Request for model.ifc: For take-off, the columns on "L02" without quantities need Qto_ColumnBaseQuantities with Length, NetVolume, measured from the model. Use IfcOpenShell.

First a look at what the model holds.

```python
import ifcopenshell
import ifcopenshell.util.element
import ifcopenshell.util.unit

model = ifcopenshell.open("model.ifc")
print(model.schema)
for unit_type in ("LENGTHUNIT", "AREAUNIT", "VOLUMEUNIT"):
    print(unit_type, ifcopenshell.util.unit.calculate_unit_scale(model, unit_type))
storey = next(s for s in model.by_type("IfcBuildingStorey") if s.Name == "L02")
columns = [e for e in ifcopenshell.util.element.get_decomposition(storey) if e.is_a("IfcColumn")]
for e in sorted(columns, key=lambda e: e.id()):
    print(e.id(), e.is_a(), e.Name, list(ifcopenshell.util.element.get_psets(e, qtos_only=True)), sep=" | ")
```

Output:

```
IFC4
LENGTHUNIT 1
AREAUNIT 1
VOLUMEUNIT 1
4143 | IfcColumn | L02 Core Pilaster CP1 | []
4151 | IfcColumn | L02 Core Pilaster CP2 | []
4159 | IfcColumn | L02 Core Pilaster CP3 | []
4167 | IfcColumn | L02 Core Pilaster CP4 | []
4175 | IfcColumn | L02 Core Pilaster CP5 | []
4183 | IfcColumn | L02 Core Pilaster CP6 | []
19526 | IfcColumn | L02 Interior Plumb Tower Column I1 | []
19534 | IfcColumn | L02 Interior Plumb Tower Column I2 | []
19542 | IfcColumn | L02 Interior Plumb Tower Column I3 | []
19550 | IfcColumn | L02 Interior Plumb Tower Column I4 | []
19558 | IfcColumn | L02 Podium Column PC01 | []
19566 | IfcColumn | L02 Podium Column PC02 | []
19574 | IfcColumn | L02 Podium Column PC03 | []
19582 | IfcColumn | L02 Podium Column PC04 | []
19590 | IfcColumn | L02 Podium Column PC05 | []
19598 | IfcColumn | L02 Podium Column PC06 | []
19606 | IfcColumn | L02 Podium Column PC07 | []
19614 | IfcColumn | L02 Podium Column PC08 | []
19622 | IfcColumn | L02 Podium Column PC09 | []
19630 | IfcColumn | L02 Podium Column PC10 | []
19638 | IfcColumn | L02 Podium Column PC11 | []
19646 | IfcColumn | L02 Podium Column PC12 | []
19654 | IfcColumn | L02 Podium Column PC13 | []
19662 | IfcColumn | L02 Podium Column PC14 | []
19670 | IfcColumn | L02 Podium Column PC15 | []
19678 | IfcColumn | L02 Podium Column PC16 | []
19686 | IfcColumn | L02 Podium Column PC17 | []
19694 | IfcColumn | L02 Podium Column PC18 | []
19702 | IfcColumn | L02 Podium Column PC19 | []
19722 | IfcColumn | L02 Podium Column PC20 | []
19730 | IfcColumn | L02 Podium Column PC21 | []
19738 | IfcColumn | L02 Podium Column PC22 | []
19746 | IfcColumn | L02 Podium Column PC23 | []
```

```python
import ifcopenshell
import ifcopenshell.api.pset
import ifcopenshell.geom
import ifcopenshell.util.element
import ifcopenshell.util.shape
import ifcopenshell.util.unit

model = ifcopenshell.open("model.ifc")
unit_scale = ifcopenshell.util.unit.calculate_unit_scale(model)
volume_scale = ifcopenshell.util.unit.calculate_unit_scale(model, "VOLUMEUNIT")
settings = ifcopenshell.geom.settings()

storey = next(s for s in model.by_type("IfcBuildingStorey") if s.Name == "L02")
columns = [e for e in ifcopenshell.util.element.get_decomposition(storey) if e.is_a("IfcColumn")]

for e in sorted(columns, key=lambda e: e.id()):
    if ifcopenshell.util.element.get_psets(e, qtos_only=True, should_inherit=False):
        continue
    # Geometry comes back in metres, in the element's own axes.
    shape = ifcopenshell.geom.create_shape(settings, e)
    values = {
        "Length": ifcopenshell.util.shape.get_z(shape.geometry) / unit_scale,
        "NetVolume": ifcopenshell.util.shape.get_volume(shape.geometry) / volume_scale,
    }
    qto = ifcopenshell.api.pset.add_qto(model, product=e, name="Qto_ColumnBaseQuantities")
    ifcopenshell.api.pset.edit_qto(model, qto=qto, properties=values)
    print(e.id(), {k: round(v, 3) for k, v in values.items()})

model.write("model_rev.ifc")
```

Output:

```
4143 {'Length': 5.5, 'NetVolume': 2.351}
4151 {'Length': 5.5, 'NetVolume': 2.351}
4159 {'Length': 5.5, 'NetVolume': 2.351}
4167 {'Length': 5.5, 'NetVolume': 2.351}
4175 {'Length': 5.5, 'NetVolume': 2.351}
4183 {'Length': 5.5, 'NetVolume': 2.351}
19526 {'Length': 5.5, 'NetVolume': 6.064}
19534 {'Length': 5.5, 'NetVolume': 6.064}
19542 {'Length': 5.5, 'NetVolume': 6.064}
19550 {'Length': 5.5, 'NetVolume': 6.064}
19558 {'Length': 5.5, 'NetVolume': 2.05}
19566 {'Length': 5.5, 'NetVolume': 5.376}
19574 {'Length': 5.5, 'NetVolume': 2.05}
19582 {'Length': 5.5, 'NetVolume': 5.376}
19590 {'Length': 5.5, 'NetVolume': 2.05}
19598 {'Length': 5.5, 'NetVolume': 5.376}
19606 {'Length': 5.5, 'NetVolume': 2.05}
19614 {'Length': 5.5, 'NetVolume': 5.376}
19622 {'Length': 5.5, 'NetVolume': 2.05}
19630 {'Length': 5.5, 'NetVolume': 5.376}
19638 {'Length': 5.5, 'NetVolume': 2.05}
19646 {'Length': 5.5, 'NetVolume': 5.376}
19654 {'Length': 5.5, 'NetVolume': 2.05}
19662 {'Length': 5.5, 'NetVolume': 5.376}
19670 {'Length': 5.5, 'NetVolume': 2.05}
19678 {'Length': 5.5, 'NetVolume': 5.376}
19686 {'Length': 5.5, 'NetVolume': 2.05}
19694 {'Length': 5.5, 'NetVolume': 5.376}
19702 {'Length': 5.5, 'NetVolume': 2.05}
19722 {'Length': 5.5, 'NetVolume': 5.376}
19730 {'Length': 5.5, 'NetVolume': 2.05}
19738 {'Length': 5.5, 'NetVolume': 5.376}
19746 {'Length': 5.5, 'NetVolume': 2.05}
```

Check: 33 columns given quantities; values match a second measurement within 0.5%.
